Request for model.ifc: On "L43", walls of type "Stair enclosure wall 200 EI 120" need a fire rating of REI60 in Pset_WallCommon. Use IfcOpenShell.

First a look at what the model holds.

```python
import ifcopenshell
import ifcopenshell.util.element

model = ifcopenshell.open("model.ifc")
print(model.schema)
storey = next(s for s in model.by_type("IfcBuildingStorey") if s.Name == "L43")
walls = [e for e in ifcopenshell.util.element.get_decomposition(storey) if e.is_a("IfcWall")]
seen = {}
for e in walls:
    element_type = ifcopenshell.util.element.get_type(e)
    key = (element_type.Name if element_type != e and element_type else None, ifcopenshell.util.element.get_pset(e, "Pset_WallCommon", "FireRating"))
    seen[key] = seen.get(key, 0) + 1
for (name, value), count in sorted(seen.items(), key=str):
    print(count, "x", name, "|", value)
```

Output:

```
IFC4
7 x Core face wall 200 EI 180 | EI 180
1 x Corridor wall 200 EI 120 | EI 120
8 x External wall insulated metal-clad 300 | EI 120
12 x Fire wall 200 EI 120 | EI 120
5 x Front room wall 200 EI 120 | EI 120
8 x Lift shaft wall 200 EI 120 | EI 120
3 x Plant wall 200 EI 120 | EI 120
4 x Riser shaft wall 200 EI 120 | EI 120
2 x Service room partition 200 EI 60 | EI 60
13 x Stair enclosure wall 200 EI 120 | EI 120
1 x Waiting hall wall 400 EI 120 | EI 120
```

```python
import ifcopenshell
import ifcopenshell.api.pset
import ifcopenshell.util.element

model = ifcopenshell.open("model.ifc")

storey = next(s for s in model.by_type("IfcBuildingStorey") if s.Name == "L43")
walls = [e for e in ifcopenshell.util.element.get_decomposition(storey) if e.is_a("IfcWall")]

count = 0
for e in walls:
    element_type = ifcopenshell.util.element.get_type(e)
    if element_type in (None, e) or element_type.Name != "Stair enclosure wall 200 EI 120":
        continue
    found = ifcopenshell.util.element.get_pset(e, "Pset_WallCommon", should_inherit=False)
    if found:
        pset = model.by_id(found["id"])
        if len(ifcopenshell.util.element.get_elements_by_pset(pset)) > 1:
            pset = ifcopenshell.api.pset.unshare_pset(model, products=[e], pset=pset)[0]
    else:
        pset = ifcopenshell.api.pset.add_pset(model, product=e, name="Pset_WallCommon")
    ifcopenshell.api.pset.edit_pset(model, pset=pset, properties={"FireRating": "REI60"})
    count += 1

print(count, "walls updated")

model.write("model-out.ifc")
```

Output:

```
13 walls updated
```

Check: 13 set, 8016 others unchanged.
